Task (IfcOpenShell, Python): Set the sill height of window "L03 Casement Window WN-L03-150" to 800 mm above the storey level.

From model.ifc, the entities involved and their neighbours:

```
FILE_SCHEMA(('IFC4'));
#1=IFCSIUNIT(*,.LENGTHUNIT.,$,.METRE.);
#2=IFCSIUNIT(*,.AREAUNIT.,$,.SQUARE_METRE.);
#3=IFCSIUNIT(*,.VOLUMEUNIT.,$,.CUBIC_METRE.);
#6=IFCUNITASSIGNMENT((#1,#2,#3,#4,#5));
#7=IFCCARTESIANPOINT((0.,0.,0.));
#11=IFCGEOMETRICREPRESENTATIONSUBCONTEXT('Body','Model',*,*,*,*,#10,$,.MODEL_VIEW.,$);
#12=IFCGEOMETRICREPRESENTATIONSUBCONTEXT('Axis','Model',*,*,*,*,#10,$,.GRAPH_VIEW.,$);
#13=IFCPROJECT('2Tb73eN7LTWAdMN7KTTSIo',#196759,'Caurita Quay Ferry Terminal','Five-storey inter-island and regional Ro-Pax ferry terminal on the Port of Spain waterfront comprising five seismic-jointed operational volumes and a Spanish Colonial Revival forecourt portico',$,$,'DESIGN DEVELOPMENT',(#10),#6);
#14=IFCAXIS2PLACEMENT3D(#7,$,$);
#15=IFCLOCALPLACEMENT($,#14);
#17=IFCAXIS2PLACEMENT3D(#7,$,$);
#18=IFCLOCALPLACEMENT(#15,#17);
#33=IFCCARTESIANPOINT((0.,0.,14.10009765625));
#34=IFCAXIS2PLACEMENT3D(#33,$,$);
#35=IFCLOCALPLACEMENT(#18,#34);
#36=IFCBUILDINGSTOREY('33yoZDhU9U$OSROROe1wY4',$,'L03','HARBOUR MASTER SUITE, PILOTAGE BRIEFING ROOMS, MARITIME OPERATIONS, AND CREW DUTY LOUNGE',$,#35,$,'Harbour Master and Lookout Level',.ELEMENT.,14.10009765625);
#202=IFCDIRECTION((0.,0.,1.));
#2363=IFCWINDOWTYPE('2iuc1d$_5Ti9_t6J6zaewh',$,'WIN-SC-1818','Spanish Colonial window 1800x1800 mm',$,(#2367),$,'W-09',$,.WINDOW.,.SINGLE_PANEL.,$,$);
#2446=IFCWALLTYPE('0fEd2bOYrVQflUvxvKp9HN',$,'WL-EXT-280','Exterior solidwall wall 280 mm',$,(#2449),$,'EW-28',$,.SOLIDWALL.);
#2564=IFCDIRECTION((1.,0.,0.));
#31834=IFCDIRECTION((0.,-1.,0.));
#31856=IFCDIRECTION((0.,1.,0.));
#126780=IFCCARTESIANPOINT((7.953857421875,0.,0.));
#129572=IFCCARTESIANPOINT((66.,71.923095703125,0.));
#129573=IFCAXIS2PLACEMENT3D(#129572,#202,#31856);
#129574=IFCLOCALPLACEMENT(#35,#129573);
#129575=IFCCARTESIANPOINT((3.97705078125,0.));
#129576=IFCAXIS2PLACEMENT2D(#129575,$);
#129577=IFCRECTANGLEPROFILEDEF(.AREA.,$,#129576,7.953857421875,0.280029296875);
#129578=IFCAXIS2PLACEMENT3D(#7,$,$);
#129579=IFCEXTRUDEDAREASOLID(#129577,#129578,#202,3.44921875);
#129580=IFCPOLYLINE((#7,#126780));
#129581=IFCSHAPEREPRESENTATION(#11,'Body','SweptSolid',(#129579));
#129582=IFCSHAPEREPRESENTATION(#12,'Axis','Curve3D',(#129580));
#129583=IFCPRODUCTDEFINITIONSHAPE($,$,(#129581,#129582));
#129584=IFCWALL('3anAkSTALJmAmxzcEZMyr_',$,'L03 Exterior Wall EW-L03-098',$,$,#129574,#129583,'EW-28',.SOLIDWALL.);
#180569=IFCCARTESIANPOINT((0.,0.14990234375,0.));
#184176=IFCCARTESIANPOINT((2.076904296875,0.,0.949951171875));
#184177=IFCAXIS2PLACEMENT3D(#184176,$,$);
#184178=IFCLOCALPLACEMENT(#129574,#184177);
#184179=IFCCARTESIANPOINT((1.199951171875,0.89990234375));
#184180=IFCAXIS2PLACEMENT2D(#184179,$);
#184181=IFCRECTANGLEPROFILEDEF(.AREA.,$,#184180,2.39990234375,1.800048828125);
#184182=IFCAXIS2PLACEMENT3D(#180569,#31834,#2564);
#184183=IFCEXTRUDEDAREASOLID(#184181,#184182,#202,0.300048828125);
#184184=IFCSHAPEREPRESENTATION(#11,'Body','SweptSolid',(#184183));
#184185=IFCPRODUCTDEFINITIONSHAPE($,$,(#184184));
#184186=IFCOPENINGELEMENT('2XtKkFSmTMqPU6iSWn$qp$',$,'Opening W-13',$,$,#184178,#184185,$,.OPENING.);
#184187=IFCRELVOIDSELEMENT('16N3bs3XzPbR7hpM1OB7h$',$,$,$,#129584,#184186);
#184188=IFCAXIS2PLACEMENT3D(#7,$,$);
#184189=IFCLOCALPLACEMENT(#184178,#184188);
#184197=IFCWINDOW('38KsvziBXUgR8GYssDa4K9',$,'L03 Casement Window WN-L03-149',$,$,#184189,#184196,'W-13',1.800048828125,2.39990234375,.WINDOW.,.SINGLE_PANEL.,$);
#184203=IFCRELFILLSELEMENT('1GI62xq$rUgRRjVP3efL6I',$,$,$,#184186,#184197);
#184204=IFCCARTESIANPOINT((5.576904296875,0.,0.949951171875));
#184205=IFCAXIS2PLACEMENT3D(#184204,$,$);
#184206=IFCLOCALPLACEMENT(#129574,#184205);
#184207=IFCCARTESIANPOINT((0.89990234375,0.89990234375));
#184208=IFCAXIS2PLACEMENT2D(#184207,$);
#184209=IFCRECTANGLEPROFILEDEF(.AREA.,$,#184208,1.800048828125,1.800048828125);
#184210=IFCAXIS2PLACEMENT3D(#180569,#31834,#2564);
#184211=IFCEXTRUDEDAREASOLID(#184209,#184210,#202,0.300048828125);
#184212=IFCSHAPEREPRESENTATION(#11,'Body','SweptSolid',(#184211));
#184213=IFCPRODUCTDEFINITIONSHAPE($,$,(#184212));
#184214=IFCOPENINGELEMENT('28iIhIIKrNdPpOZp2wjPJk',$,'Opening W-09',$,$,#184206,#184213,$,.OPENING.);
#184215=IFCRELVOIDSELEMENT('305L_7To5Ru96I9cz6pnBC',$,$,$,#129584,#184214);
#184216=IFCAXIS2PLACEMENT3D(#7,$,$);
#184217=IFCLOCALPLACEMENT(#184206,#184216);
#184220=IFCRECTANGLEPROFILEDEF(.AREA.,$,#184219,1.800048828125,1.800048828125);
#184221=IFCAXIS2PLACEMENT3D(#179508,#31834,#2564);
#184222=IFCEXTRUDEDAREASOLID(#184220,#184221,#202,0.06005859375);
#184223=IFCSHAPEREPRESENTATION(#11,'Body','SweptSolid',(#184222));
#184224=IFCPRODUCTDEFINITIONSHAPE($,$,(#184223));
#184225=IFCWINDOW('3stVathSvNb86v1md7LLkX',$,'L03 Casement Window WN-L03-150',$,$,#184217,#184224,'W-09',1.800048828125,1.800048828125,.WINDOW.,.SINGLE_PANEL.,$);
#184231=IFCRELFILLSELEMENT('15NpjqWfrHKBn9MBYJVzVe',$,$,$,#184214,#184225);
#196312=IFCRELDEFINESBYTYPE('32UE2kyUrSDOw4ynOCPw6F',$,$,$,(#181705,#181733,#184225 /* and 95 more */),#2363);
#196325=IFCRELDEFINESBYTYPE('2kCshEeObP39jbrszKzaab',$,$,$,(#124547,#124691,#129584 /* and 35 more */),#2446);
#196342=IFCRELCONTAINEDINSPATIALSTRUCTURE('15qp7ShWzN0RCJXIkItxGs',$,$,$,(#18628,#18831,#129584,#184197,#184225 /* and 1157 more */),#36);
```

```python
import numpy as np
import ifcopenshell
import ifcopenshell.api.geometry
import ifcopenshell.geom
import ifcopenshell.util.element
import ifcopenshell.util.placement
import ifcopenshell.util.shape
import ifcopenshell.util.unit

model = ifcopenshell.open("model.ifc")
unit_scale = ifcopenshell.util.unit.calculate_unit_scale(model)

window = model.by_id(184225)
opening = window.FillsVoids[0].RelatingOpeningElement
storey = ifcopenshell.util.element.get_container(window, ifc_class="IfcBuildingStorey")
level = ifcopenshell.util.placement.get_local_placement(storey.ObjectPlacement)[2, 3]

# The opening's origin need not be at the sill, so measure its lowest point.
shape = ifcopenshell.geom.create_shape(ifcopenshell.geom.settings(), opening)
bottom = ifcopenshell.util.shape.get_shape_bottom_elevation(shape, shape.geometry) / unit_scale
dz = level + 0.8 / unit_scale - bottom

shift = np.array([0.0, 0.0, dz])
# The window is placed relative to its opening, so it follows when the opening moves.
matrix = ifcopenshell.util.placement.get_local_placement(opening.ObjectPlacement)
matrix[:3, 3] += shift
ifcopenshell.api.geometry.edit_object_placement(
    model, product=opening, matrix=matrix, is_si=False, should_transform_children=True
)

print(f"moved by {dz * unit_scale:+.3f} m")

model.write("model_edited.ifc")
```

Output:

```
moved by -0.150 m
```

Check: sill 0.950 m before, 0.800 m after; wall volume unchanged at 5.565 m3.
